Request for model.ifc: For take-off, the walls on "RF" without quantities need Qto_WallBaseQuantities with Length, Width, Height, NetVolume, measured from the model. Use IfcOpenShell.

First a look at what the model holds.

```python
import ifcopenshell
import ifcopenshell.util.element
import ifcopenshell.util.unit

model = ifcopenshell.open("model.ifc")
print(model.schema)
for unit_type in ("LENGTHUNIT", "AREAUNIT", "VOLUMEUNIT"):
    print(unit_type, ifcopenshell.util.unit.calculate_unit_scale(model, unit_type))
storey = next(s for s in model.by_type("IfcBuildingStorey") if s.Name == "RF")
walls = [e for e in ifcopenshell.util.element.get_decomposition(storey) if e.is_a("IfcWall")]
for e in sorted(walls, key=lambda e: e.id()):
    print(e.id(), e.is_a(), e.Name, list(ifcopenshell.util.element.get_psets(e, qtos_only=True)), sep=" | ")
```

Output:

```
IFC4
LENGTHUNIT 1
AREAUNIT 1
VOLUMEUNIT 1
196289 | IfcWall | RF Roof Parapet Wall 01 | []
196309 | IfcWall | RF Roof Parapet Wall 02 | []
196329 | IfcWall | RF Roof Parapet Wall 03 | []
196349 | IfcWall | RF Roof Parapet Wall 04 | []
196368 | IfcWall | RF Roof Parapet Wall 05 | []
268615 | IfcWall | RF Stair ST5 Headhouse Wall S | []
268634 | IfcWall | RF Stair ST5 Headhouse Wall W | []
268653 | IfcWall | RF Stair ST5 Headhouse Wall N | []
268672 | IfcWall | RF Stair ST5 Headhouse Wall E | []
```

```python
import ifcopenshell
import ifcopenshell.api.pset
import ifcopenshell.geom
import ifcopenshell.util.element
import ifcopenshell.util.shape
import ifcopenshell.util.unit

model = ifcopenshell.open("model.ifc")
unit_scale = ifcopenshell.util.unit.calculate_unit_scale(model)
volume_scale = ifcopenshell.util.unit.calculate_unit_scale(model, "VOLUMEUNIT")
settings = ifcopenshell.geom.settings()

storey = next(s for s in model.by_type("IfcBuildingStorey") if s.Name == "RF")
walls = [e for e in ifcopenshell.util.element.get_decomposition(storey) if e.is_a("IfcWall")]

for e in sorted(walls, key=lambda e: e.id()):
    if ifcopenshell.util.element.get_psets(e, qtos_only=True, should_inherit=False):
        continue
    # Geometry comes back in metres, in the element's own axes.
    shape = ifcopenshell.geom.create_shape(settings, e)
    values = {
        "Length": ifcopenshell.util.shape.get_x(shape.geometry) / unit_scale,
        "Width": ifcopenshell.util.shape.get_y(shape.geometry) / unit_scale,
        "Height": ifcopenshell.util.shape.get_z(shape.geometry) / unit_scale,
        "NetVolume": ifcopenshell.util.shape.get_volume(shape.geometry) / volume_scale,
    }
    qto = ifcopenshell.api.pset.add_qto(model, product=e, name="Qto_WallBaseQuantities")
    ifcopenshell.api.pset.edit_qto(model, qto=qto, properties=values)
    print(e.id(), {k: round(v, 3) for k, v in values.items()})

model.write("model_v2.ifc")
```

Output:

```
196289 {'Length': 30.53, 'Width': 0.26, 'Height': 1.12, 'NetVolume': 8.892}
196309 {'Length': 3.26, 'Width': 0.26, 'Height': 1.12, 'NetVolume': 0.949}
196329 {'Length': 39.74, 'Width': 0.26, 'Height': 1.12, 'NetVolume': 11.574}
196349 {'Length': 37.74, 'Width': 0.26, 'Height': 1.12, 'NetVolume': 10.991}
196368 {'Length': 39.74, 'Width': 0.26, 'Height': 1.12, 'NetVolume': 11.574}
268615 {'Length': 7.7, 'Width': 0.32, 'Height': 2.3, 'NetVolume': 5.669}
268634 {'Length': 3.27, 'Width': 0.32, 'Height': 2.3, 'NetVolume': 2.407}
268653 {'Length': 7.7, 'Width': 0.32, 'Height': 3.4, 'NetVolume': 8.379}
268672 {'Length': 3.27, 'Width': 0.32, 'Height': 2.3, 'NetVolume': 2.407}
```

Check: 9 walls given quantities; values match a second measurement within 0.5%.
